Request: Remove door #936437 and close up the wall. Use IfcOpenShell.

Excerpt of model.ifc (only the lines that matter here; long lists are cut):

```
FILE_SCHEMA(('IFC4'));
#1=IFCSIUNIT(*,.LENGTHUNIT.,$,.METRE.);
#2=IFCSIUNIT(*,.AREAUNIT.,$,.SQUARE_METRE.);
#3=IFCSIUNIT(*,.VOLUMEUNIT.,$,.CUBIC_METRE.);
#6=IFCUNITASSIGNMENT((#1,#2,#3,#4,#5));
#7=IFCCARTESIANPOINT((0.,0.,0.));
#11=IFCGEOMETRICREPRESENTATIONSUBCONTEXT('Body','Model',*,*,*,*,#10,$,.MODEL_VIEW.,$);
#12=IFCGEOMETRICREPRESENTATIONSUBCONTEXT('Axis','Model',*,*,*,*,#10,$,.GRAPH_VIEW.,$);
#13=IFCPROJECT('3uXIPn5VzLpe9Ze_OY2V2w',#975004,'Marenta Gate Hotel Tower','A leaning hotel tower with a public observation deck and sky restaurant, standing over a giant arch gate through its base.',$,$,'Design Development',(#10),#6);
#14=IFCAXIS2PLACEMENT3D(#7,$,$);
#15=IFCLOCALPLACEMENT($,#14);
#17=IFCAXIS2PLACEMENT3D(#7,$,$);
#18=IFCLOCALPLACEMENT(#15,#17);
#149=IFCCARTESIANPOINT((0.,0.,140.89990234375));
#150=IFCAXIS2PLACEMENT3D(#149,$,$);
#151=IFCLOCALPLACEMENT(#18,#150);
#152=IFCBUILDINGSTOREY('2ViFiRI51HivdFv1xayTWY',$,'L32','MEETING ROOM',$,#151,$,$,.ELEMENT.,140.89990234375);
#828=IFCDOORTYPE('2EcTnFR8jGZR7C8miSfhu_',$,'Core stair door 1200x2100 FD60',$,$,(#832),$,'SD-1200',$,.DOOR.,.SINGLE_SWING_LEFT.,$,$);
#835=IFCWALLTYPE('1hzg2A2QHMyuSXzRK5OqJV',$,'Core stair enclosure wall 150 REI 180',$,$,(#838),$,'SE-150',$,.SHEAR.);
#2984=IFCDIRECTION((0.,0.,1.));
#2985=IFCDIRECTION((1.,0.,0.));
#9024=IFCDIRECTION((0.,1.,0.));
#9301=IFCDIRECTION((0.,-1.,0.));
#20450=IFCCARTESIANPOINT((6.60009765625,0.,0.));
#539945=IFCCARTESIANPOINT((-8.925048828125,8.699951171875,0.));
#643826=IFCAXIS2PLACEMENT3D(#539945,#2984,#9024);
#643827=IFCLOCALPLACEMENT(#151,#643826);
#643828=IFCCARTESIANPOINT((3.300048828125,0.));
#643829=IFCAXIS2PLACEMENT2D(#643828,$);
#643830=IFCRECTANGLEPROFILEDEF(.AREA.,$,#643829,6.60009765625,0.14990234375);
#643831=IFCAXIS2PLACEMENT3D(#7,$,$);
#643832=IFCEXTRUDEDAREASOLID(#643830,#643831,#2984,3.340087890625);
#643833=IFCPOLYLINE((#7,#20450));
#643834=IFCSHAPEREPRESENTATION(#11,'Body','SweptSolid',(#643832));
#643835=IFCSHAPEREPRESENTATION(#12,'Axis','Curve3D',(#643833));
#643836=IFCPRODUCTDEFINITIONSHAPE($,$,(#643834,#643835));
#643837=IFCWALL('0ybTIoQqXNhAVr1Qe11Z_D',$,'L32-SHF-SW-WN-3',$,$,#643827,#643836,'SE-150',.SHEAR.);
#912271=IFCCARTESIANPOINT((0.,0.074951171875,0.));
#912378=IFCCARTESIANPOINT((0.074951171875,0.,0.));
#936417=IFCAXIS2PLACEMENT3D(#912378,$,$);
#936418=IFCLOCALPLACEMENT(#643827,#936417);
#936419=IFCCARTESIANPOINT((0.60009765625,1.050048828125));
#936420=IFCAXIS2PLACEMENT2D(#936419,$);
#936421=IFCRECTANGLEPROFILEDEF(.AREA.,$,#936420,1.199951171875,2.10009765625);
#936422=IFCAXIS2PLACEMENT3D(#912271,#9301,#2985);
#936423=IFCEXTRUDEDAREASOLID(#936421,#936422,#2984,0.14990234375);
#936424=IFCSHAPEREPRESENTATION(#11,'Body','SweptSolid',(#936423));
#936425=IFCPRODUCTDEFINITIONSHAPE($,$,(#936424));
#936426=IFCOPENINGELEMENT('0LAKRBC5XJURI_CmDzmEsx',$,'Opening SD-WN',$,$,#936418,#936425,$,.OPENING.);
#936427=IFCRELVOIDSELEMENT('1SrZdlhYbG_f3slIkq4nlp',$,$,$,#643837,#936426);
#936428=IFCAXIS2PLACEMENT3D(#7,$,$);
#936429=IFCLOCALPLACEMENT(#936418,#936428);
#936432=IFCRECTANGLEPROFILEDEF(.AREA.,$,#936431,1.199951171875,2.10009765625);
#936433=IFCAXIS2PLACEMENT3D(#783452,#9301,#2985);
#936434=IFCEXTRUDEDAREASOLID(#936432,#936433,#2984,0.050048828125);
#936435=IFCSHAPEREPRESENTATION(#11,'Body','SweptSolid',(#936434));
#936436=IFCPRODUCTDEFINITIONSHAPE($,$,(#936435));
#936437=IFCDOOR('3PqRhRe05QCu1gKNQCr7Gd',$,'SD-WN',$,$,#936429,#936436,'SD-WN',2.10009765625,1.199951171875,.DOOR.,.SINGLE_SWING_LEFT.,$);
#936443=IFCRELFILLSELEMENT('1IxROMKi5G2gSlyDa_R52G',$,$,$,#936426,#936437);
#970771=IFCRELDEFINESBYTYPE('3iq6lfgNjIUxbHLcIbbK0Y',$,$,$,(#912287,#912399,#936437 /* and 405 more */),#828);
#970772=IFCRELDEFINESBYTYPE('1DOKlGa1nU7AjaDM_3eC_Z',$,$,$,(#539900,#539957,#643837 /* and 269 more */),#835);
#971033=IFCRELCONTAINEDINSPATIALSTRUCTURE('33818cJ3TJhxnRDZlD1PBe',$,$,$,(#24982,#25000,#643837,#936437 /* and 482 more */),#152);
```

```python
import ifcopenshell
import ifcopenshell.api.feature
import ifcopenshell.api.root
import ifcopenshell.geom
import ifcopenshell.util.shape

model = ifcopenshell.open("model.ifc")
settings = ifcopenshell.geom.settings()


def volume(element):
    """Net volume in cubic metres, openings subtracted."""
    shape = ifcopenshell.geom.create_shape(settings, element)
    return ifcopenshell.util.shape.get_volume(shape.geometry)


door = model.by_guid("3PqRhRe05QCu1gKNQCr7Gd")
opening = door.FillsVoids[0].RelatingOpeningElement
wall = opening.VoidsElements[0].RelatingBuildingElement
before = volume(wall)

ifcopenshell.api.root.remove_product(model, product=door)
ifcopenshell.api.feature.remove_feature(model, feature=opening)

after = volume(wall)

print(f"wall volume {before:.3f} -> {after:.3f} m3")

model.write("model-out.ifc")
```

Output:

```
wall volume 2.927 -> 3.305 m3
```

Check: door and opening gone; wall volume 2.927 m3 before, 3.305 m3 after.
